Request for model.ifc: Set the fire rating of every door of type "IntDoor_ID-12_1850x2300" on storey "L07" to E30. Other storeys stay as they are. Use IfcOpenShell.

First a look at what the model holds.

```python
import ifcopenshell
import ifcopenshell.util.element

model = ifcopenshell.open("model.ifc")
print(model.schema)
storey = next(s for s in model.by_type("IfcBuildingStorey") if s.Name == "L07")
doors = [e for e in ifcopenshell.util.element.get_decomposition(storey) if e.is_a("IfcDoor")]
seen = {}
for e in doors:
    element_type = ifcopenshell.util.element.get_type(e)
    key = (element_type.Name if element_type != e and element_type else None, ifcopenshell.util.element.get_pset(e, "Pset_DoorCommon", "FireRating"))
    seen[key] = seen.get(key, 0) + 1
for (name, value), count in sorted(seen.items(), key=str):
    print(count, "x", name, "|", value)
```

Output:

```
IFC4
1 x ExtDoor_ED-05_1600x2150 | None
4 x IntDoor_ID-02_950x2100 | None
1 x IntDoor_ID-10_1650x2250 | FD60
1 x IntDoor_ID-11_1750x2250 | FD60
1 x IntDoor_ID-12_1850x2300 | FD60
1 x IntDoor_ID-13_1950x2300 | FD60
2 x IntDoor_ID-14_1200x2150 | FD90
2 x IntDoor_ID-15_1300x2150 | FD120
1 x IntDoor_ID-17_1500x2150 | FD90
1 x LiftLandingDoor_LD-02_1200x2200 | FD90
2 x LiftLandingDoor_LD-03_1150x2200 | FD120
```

```python
import ifcopenshell
import ifcopenshell.api.pset
import ifcopenshell.util.element

model = ifcopenshell.open("model.ifc")

storey = next(s for s in model.by_type("IfcBuildingStorey") if s.Name == "L07")
doors = [e for e in ifcopenshell.util.element.get_decomposition(storey) if e.is_a("IfcDoor")]

count = 0
for e in doors:
    element_type = ifcopenshell.util.element.get_type(e)
    if element_type in (None, e) or element_type.Name != "IntDoor_ID-12_1850x2300":
        continue
    # add_pset returns the element's existing set when there is one.
    pset = ifcopenshell.api.pset.add_pset(model, product=e, name="Pset_DoorCommon")
    ifcopenshell.api.pset.edit_pset(model, pset=pset, properties={"FireRating": "E30"})
    count += 1

print(count, "doors updated")

model.write("model_edited.ifc")
```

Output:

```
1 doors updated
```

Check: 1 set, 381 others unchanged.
